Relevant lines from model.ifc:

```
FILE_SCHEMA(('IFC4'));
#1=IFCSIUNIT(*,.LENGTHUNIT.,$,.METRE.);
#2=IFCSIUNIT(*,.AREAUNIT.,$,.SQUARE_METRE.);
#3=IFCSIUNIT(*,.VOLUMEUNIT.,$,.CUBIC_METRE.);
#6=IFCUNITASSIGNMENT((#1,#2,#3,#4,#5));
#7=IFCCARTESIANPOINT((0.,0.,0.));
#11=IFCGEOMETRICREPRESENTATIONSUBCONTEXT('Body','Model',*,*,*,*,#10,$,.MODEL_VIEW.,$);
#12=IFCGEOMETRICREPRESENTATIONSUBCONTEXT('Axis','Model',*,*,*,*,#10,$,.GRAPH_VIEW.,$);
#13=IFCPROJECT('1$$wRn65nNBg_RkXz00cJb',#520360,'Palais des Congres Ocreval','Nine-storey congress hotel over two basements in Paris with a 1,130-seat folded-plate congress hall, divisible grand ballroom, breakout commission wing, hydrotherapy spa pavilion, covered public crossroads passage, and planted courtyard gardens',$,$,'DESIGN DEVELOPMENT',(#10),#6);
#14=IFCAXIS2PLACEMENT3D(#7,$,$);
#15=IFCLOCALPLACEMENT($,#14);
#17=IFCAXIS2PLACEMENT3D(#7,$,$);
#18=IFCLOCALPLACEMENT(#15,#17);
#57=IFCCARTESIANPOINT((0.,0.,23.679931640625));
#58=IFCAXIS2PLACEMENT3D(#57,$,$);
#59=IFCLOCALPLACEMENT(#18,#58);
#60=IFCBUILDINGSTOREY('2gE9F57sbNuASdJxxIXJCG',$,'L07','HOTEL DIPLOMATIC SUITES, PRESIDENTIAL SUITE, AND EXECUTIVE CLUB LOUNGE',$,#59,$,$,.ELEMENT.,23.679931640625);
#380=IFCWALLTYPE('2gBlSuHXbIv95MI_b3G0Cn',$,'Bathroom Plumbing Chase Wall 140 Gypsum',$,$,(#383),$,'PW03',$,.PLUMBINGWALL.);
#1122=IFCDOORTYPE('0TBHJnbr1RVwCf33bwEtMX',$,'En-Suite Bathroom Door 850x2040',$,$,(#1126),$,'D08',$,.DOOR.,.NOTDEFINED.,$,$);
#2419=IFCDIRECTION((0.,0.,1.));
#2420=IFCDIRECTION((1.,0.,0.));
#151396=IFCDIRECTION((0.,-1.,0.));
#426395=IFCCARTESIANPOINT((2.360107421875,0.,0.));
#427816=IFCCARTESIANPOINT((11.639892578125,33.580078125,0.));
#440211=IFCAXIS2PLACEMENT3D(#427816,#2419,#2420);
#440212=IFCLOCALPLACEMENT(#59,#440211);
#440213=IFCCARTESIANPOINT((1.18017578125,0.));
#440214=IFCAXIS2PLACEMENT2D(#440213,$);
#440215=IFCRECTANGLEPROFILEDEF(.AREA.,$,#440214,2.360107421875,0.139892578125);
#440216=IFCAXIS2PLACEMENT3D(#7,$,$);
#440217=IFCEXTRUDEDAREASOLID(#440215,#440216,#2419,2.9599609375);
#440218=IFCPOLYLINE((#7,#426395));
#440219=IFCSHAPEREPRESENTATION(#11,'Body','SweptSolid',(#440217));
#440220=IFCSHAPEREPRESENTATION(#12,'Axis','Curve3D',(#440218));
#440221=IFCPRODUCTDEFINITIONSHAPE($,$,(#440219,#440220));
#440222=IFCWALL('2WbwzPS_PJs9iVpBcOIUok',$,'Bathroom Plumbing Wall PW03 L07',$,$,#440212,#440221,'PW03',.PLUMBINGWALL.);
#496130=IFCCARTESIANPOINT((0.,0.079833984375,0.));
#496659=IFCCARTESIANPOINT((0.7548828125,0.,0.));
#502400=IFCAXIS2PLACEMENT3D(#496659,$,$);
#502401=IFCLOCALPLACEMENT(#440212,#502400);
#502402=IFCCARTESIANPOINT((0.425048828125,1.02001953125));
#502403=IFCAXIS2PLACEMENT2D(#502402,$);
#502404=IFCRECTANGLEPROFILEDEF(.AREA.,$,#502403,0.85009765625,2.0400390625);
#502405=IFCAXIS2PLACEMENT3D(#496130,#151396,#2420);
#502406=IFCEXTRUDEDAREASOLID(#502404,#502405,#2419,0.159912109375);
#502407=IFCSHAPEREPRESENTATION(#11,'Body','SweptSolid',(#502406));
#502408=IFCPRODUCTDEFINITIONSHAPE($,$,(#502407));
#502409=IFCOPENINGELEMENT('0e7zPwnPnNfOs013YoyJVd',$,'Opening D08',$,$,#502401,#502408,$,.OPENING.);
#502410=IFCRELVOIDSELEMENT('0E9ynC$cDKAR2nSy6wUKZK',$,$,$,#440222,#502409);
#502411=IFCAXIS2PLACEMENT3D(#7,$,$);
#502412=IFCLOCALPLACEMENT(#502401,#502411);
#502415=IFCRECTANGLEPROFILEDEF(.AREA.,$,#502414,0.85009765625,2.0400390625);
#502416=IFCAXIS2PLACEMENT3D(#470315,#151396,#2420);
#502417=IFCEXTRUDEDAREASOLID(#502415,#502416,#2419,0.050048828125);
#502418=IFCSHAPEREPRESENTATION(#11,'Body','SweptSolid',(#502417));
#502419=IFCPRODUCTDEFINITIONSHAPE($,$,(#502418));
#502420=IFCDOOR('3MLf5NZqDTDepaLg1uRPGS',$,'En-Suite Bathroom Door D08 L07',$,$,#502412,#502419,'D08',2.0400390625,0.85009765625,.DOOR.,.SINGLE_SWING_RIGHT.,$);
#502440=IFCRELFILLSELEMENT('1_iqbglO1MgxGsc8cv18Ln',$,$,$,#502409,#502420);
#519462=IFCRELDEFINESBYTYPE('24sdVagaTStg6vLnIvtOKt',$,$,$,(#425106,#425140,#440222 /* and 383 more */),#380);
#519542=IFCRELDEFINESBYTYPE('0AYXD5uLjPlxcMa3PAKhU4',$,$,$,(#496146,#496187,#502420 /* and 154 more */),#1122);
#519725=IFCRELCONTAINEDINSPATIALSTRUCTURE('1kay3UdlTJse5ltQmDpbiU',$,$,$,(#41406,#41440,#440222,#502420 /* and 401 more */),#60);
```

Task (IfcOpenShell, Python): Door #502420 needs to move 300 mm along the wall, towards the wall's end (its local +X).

```python
import ifcopenshell
import ifcopenshell.api.geometry
import ifcopenshell.util.placement
import ifcopenshell.util.unit

model = ifcopenshell.open("model.ifc")
unit_scale = ifcopenshell.util.unit.calculate_unit_scale(model)

door = model.by_id(502420)
opening = door.FillsVoids[0].RelatingOpeningElement
wall = opening.VoidsElements[0].RelatingBuildingElement

wall_matrix = ifcopenshell.util.placement.get_local_placement(wall.ObjectPlacement)
shift = wall_matrix[:3, 0] * 0.3 / unit_scale
before = ifcopenshell.util.placement.get_local_placement(door.ObjectPlacement)[:3, 3].copy()

# The door is placed relative to its opening, so it follows when the opening moves.
matrix = ifcopenshell.util.placement.get_local_placement(opening.ObjectPlacement)
matrix[:3, 3] += shift
ifcopenshell.api.geometry.edit_object_placement(
    model, product=opening, matrix=matrix, is_si=False, should_transform_children=True
)

after = ifcopenshell.util.placement.get_local_placement(door.ObjectPlacement)[:3, 3]
print("door moved by", (after - before).round(3) + 0.0)

model.write("model_rev.ifc")
```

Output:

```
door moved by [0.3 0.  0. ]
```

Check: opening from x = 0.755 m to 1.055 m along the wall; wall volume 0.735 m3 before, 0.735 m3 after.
